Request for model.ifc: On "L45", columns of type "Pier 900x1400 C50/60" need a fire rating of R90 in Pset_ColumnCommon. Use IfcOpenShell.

First a look at what the model holds.

```python
import ifcopenshell
import ifcopenshell.util.element

model = ifcopenshell.open("model.ifc")
print(model.schema)
storey = next(s for s in model.by_type("IfcBuildingStorey") if s.Name == "L45")
columns = [e for e in ifcopenshell.util.element.get_decomposition(storey) if e.is_a("IfcColumn")]
seen = {}
for e in columns:
    element_type = ifcopenshell.util.element.get_type(e)
    key = (element_type.Name if element_type != e and element_type else None, ifcopenshell.util.element.get_pset(e, "Pset_ColumnCommon", "FireRating"))
    seen[key] = seen.get(key, 0) + 1
for (name, value), count in sorted(seen.items(), key=str):
    print(count, "x", name, "|", value)
```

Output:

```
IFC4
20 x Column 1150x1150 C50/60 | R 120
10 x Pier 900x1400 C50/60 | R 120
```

```python
import ifcopenshell
import ifcopenshell.api.pset
import ifcopenshell.util.element

model = ifcopenshell.open("model.ifc")

storey = next(s for s in model.by_type("IfcBuildingStorey") if s.Name == "L45")
columns = [e for e in ifcopenshell.util.element.get_decomposition(storey) if e.is_a("IfcColumn")]

count = 0
for e in columns:
    element_type = ifcopenshell.util.element.get_type(e)
    if element_type in (None, e) or element_type.Name != "Pier 900x1400 C50/60":
        continue
    found = ifcopenshell.util.element.get_pset(e, "Pset_ColumnCommon", should_inherit=False)
    if found:
        pset = model.by_id(found["id"])
        if len(ifcopenshell.util.element.get_elements_by_pset(pset)) > 1:
            pset = ifcopenshell.api.pset.unshare_pset(model, products=[e], pset=pset)[0]
    else:
        pset = ifcopenshell.api.pset.add_pset(model, product=e, name="Pset_ColumnCommon")
    ifcopenshell.api.pset.edit_pset(model, pset=pset, properties={"FireRating": "R90"})
    count += 1

print(count, "columns updated")

model.write("model_edited.ifc")
```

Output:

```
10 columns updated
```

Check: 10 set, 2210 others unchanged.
